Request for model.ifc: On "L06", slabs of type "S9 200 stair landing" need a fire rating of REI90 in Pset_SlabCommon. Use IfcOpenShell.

First a look at what the model holds.

```python
import ifcopenshell
import ifcopenshell.util.element

model = ifcopenshell.open("model.ifc")
print(model.schema)
storey = next(s for s in model.by_type("IfcBuildingStorey") if s.Name == "L06")
slabs = [e for e in ifcopenshell.util.element.get_decomposition(storey) if e.is_a("IfcSlab")]
seen = {}
for e in slabs:
    element_type = ifcopenshell.util.element.get_type(e)
    key = (element_type.Name if element_type != e and element_type else None, ifcopenshell.util.element.get_pset(e, "Pset_SlabCommon", "FireRating"))
    seen[key] = seen.get(key, 0) + 1
for (name, value), count in sorted(seen.items(), key=str):
    print(count, "x", name, "|", value)
```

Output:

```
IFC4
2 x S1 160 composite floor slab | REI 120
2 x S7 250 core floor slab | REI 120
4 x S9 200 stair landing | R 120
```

```python
import ifcopenshell
import ifcopenshell.api.pset
import ifcopenshell.util.element

model = ifcopenshell.open("model.ifc")

storey = next(s for s in model.by_type("IfcBuildingStorey") if s.Name == "L06")
slabs = [e for e in ifcopenshell.util.element.get_decomposition(storey) if e.is_a("IfcSlab")]

count = 0
for e in slabs:
    element_type = ifcopenshell.util.element.get_type(e)
    if element_type in (None, e) or element_type.Name != "S9 200 stair landing":
        continue
    # add_pset returns the element's existing set when there is one.
    pset = ifcopenshell.api.pset.add_pset(model, product=e, name="Pset_SlabCommon")
    ifcopenshell.api.pset.edit_pset(model, pset=pset, properties={"FireRating": "REI90"})
    count += 1

print(count, "slabs updated")

model.write("model_v2.ifc")
```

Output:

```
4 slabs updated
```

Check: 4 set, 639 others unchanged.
